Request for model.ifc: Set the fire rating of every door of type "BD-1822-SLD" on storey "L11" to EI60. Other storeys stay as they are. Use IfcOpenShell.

First a look at what the model holds.

```python
import ifcopenshell
import ifcopenshell.util.element

model = ifcopenshell.open("model.ifc")
print(model.schema)
storey = next(s for s in model.by_type("IfcBuildingStorey") if s.Name == "L11")
doors = [e for e in ifcopenshell.util.element.get_decomposition(storey) if e.is_a("IfcDoor")]
seen = {}
for e in doors:
    element_type = ifcopenshell.util.element.get_type(e)
    key = (element_type.Name if element_type != e and element_type else None, ifcopenshell.util.element.get_pset(e, "Pset_DoorCommon", "FireRating"))
    seen[key] = seen.get(key, 0) + 1
for (name, value), count in sorted(seen.items(), key=str):
    print(count, "x", name, "|", value)
```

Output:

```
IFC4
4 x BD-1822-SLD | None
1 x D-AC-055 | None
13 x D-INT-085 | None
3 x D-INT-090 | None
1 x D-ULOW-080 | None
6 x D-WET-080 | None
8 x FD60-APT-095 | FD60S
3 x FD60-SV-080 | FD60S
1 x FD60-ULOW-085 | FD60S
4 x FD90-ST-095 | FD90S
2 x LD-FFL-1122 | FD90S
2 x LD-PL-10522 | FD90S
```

```python
import ifcopenshell
import ifcopenshell.api.pset
import ifcopenshell.util.element

model = ifcopenshell.open("model.ifc")

storey = next(s for s in model.by_type("IfcBuildingStorey") if s.Name == "L11")
doors = [e for e in ifcopenshell.util.element.get_decomposition(storey) if e.is_a("IfcDoor")]

count = 0
for e in doors:
    element_type = ifcopenshell.util.element.get_type(e)
    if element_type in (None, e) or element_type.Name != "BD-1822-SLD":
        continue
    found = ifcopenshell.util.element.get_pset(e, "Pset_DoorCommon", should_inherit=False)
    if found:
        pset = model.by_id(found["id"])
        if len(ifcopenshell.util.element.get_elements_by_pset(pset)) > 1:
            pset = ifcopenshell.api.pset.unshare_pset(model, products=[e], pset=pset)[0]
    else:
        pset = ifcopenshell.api.pset.add_pset(model, product=e, name="Pset_DoorCommon")
    ifcopenshell.api.pset.edit_pset(model, pset=pset, properties={"FireRating": "EI60"})
    count += 1

print(count, "doors updated")

model.write("model_v2.ifc")
```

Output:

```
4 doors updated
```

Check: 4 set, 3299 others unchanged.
